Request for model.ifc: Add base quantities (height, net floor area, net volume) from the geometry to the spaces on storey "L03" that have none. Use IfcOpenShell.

First a look at what the model holds.

```python
import ifcopenshell
import ifcopenshell.util.element
import ifcopenshell.util.unit

model = ifcopenshell.open("model.ifc")
print(model.schema)
for unit_type in ("LENGTHUNIT", "AREAUNIT", "VOLUMEUNIT"):
    print(unit_type, ifcopenshell.util.unit.calculate_unit_scale(model, unit_type))
storey = next(s for s in model.by_type("IfcBuildingStorey") if s.Name == "L03")
spaces = [e for e in ifcopenshell.util.element.get_decomposition(storey) if e.is_a("IfcSpace")]
for e in sorted(spaces, key=lambda e: e.id()):
    print(e.id(), e.is_a(), e.Name, list(ifcopenshell.util.element.get_psets(e, qtos_only=True)), sep=" | ")
```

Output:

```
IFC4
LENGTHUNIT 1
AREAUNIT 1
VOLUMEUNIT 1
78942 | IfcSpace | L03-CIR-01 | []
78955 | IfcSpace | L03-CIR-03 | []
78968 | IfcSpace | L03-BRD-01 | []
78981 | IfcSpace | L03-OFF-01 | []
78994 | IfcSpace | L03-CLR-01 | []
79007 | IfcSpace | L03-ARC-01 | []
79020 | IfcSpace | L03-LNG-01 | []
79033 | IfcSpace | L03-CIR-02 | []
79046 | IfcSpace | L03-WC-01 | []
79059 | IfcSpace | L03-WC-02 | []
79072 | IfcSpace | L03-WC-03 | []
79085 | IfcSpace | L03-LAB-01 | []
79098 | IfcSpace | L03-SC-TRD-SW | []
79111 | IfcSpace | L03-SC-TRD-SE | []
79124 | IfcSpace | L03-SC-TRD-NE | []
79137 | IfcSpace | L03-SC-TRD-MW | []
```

```python
import ifcopenshell
import ifcopenshell.api.pset
import ifcopenshell.geom
import ifcopenshell.util.element
import ifcopenshell.util.shape
import ifcopenshell.util.unit

model = ifcopenshell.open("model.ifc")
unit_scale = ifcopenshell.util.unit.calculate_unit_scale(model)
area_scale = ifcopenshell.util.unit.calculate_unit_scale(model, "AREAUNIT")
volume_scale = ifcopenshell.util.unit.calculate_unit_scale(model, "VOLUMEUNIT")
settings = ifcopenshell.geom.settings()

storey = next(s for s in model.by_type("IfcBuildingStorey") if s.Name == "L03")
spaces = [e for e in ifcopenshell.util.element.get_decomposition(storey) if e.is_a("IfcSpace")]

for e in sorted(spaces, key=lambda e: e.id()):
    if ifcopenshell.util.element.get_psets(e, qtos_only=True, should_inherit=False):
        continue
    # Geometry comes back in metres, in the element's own axes.
    shape = ifcopenshell.geom.create_shape(settings, e)
    values = {
        "Height": ifcopenshell.util.shape.get_z(shape.geometry) / unit_scale,
        "NetFloorArea": ifcopenshell.util.shape.get_footprint_area(shape.geometry) / area_scale,
        "NetVolume": ifcopenshell.util.shape.get_volume(shape.geometry) / volume_scale,
    }
    qto = ifcopenshell.api.pset.add_qto(model, product=e, name="Qto_SpaceBaseQuantities")
    ifcopenshell.api.pset.edit_qto(model, qto=qto, properties=values)
    print(e.id(), {k: round(v, 3) for k, v in values.items()})

model.write("model_edited.ifc")
```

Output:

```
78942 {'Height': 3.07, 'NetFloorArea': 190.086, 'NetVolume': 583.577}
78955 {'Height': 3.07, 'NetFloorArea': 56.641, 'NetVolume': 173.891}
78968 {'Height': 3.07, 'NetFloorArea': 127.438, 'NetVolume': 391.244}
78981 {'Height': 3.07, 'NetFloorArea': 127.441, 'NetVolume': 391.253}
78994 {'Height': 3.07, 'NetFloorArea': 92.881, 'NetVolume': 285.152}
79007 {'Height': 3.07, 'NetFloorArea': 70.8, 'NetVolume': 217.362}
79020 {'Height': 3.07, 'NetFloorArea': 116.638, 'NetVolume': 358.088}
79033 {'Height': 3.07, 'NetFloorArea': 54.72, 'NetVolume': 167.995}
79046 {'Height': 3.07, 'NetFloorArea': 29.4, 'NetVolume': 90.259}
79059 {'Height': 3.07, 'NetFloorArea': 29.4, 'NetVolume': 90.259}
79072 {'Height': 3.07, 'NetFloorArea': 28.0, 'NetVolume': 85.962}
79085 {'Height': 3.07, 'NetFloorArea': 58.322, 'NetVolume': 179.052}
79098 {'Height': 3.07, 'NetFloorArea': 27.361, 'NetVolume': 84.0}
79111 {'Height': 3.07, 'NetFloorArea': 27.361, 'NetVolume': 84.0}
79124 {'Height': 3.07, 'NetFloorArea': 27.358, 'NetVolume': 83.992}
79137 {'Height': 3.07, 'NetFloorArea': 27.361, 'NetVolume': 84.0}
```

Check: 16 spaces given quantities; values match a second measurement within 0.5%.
